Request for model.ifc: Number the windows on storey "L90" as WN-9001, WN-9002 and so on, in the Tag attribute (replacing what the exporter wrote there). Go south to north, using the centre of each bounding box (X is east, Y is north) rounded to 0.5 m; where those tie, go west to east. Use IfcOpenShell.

First a look at what the model holds.

```python
import ifcopenshell
import ifcopenshell.util.element
import ifcopenshell.util.placement

model = ifcopenshell.open("model.ifc")
print(model.schema)
storey = next(s for s in model.by_type("IfcBuildingStorey") if s.Name == "L90")
windows = [e for e in ifcopenshell.util.element.get_decomposition(storey) if e.is_a("IfcWindow")]
for e in sorted(windows, key=lambda e: e.id()):
    origin = ifcopenshell.util.placement.get_local_placement(e.ObjectPlacement)[:3, 3]
    print(e.id(), e.Tag, e.Name, origin.round(2) + 0.0, sep=" | ")
```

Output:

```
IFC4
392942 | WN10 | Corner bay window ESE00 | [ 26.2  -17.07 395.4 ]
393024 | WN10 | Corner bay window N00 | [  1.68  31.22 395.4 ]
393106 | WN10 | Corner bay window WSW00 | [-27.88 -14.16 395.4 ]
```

```python
import ifcopenshell
import ifcopenshell.geom
import ifcopenshell.util.element
import ifcopenshell.util.shape

model = ifcopenshell.open("model.ifc")
settings = ifcopenshell.geom.settings()
settings.set("use-world-coords", True)


def centre(element):
    shape = ifcopenshell.geom.create_shape(settings, element)
    return ifcopenshell.util.shape.get_bbox_centroid(shape.geometry)


storey = next(s for s in model.by_type("IfcBuildingStorey") if s.Name == "L90")
windows = [e for e in ifcopenshell.util.element.get_decomposition(storey) if e.is_a("IfcWindow")]

# Insertion points can sit at a corner or the storey origin, so sort by the geometry (in metres).
centres = {e: centre(e) for e in windows}
windows.sort(key=lambda e: (round(centres[e][1] / 0.5), centres[e][0]))

for i, e in enumerate(windows, start=1):
    number = f"WN-90{i:02d}"
    e.Tag = number
    print(e.id(), number)

model.write("model_rev.ifc")
```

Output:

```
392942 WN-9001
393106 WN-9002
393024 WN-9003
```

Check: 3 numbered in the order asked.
